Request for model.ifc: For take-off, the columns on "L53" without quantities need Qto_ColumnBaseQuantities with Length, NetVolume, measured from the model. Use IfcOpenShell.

First a look at what the model holds.

```python
import ifcopenshell
import ifcopenshell.util.element
import ifcopenshell.util.unit

model = ifcopenshell.open("model.ifc")
print(model.schema)
for unit_type in ("LENGTHUNIT", "AREAUNIT", "VOLUMEUNIT"):
    print(unit_type, ifcopenshell.util.unit.calculate_unit_scale(model, unit_type))
storey = next(s for s in model.by_type("IfcBuildingStorey") if s.Name == "L53")
columns = [e for e in ifcopenshell.util.element.get_decomposition(storey) if e.is_a("IfcColumn")]
for e in sorted(columns, key=lambda e: e.id()):
    print(e.id(), e.is_a(), e.Name, list(ifcopenshell.util.element.get_psets(e, qtos_only=True)), sep=" | ")
```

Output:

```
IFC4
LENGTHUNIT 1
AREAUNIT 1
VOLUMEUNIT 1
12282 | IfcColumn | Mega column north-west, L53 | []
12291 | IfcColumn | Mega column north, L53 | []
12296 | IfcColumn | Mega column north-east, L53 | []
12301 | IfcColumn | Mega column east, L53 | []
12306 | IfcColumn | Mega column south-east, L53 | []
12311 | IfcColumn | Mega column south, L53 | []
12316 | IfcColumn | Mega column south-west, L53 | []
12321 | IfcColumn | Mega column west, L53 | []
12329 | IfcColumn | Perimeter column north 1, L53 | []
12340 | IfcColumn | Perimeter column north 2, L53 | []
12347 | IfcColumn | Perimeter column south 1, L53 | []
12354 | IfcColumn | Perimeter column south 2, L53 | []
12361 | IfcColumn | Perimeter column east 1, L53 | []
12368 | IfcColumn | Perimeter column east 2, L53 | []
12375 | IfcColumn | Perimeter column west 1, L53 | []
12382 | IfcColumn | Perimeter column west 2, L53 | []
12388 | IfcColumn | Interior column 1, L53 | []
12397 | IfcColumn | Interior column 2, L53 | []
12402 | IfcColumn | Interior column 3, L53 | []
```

```python
import ifcopenshell
import ifcopenshell.api.pset
import ifcopenshell.geom
import ifcopenshell.util.element
import ifcopenshell.util.shape
import ifcopenshell.util.unit

model = ifcopenshell.open("model.ifc")
unit_scale = ifcopenshell.util.unit.calculate_unit_scale(model)
volume_scale = ifcopenshell.util.unit.calculate_unit_scale(model, "VOLUMEUNIT")
settings = ifcopenshell.geom.settings()

storey = next(s for s in model.by_type("IfcBuildingStorey") if s.Name == "L53")
columns = [e for e in ifcopenshell.util.element.get_decomposition(storey) if e.is_a("IfcColumn")]

for e in sorted(columns, key=lambda e: e.id()):
    if ifcopenshell.util.element.get_psets(e, qtos_only=True, should_inherit=False):
        continue
    # Geometry comes back in metres, in the element's own axes.
    shape = ifcopenshell.geom.create_shape(settings, e)
    values = {
        "Length": ifcopenshell.util.shape.get_z(shape.geometry) / unit_scale,
        "NetVolume": ifcopenshell.util.shape.get_volume(shape.geometry) / volume_scale,
    }
    qto = ifcopenshell.api.pset.add_qto(model, product=e, name="Qto_ColumnBaseQuantities")
    ifcopenshell.api.pset.edit_qto(model, qto=qto, properties=values)
    print(e.id(), {k: round(v, 3) for k, v in values.items()})

model.write("model_edited.ifc")
```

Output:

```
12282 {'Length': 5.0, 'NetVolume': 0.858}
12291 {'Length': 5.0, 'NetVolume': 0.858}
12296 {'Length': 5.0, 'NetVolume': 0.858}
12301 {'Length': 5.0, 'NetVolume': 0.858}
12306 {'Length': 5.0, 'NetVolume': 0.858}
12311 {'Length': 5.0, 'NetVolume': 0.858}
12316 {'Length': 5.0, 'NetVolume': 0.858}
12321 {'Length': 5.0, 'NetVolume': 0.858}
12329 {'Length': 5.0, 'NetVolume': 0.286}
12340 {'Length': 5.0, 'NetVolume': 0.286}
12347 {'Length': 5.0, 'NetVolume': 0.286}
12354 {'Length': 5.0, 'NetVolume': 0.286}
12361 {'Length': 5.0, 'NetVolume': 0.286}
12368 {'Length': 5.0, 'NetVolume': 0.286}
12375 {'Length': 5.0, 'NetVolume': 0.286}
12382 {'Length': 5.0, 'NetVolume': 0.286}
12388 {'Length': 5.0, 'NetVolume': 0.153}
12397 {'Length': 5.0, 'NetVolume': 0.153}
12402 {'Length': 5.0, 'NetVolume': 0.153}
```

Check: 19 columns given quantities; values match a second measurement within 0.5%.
